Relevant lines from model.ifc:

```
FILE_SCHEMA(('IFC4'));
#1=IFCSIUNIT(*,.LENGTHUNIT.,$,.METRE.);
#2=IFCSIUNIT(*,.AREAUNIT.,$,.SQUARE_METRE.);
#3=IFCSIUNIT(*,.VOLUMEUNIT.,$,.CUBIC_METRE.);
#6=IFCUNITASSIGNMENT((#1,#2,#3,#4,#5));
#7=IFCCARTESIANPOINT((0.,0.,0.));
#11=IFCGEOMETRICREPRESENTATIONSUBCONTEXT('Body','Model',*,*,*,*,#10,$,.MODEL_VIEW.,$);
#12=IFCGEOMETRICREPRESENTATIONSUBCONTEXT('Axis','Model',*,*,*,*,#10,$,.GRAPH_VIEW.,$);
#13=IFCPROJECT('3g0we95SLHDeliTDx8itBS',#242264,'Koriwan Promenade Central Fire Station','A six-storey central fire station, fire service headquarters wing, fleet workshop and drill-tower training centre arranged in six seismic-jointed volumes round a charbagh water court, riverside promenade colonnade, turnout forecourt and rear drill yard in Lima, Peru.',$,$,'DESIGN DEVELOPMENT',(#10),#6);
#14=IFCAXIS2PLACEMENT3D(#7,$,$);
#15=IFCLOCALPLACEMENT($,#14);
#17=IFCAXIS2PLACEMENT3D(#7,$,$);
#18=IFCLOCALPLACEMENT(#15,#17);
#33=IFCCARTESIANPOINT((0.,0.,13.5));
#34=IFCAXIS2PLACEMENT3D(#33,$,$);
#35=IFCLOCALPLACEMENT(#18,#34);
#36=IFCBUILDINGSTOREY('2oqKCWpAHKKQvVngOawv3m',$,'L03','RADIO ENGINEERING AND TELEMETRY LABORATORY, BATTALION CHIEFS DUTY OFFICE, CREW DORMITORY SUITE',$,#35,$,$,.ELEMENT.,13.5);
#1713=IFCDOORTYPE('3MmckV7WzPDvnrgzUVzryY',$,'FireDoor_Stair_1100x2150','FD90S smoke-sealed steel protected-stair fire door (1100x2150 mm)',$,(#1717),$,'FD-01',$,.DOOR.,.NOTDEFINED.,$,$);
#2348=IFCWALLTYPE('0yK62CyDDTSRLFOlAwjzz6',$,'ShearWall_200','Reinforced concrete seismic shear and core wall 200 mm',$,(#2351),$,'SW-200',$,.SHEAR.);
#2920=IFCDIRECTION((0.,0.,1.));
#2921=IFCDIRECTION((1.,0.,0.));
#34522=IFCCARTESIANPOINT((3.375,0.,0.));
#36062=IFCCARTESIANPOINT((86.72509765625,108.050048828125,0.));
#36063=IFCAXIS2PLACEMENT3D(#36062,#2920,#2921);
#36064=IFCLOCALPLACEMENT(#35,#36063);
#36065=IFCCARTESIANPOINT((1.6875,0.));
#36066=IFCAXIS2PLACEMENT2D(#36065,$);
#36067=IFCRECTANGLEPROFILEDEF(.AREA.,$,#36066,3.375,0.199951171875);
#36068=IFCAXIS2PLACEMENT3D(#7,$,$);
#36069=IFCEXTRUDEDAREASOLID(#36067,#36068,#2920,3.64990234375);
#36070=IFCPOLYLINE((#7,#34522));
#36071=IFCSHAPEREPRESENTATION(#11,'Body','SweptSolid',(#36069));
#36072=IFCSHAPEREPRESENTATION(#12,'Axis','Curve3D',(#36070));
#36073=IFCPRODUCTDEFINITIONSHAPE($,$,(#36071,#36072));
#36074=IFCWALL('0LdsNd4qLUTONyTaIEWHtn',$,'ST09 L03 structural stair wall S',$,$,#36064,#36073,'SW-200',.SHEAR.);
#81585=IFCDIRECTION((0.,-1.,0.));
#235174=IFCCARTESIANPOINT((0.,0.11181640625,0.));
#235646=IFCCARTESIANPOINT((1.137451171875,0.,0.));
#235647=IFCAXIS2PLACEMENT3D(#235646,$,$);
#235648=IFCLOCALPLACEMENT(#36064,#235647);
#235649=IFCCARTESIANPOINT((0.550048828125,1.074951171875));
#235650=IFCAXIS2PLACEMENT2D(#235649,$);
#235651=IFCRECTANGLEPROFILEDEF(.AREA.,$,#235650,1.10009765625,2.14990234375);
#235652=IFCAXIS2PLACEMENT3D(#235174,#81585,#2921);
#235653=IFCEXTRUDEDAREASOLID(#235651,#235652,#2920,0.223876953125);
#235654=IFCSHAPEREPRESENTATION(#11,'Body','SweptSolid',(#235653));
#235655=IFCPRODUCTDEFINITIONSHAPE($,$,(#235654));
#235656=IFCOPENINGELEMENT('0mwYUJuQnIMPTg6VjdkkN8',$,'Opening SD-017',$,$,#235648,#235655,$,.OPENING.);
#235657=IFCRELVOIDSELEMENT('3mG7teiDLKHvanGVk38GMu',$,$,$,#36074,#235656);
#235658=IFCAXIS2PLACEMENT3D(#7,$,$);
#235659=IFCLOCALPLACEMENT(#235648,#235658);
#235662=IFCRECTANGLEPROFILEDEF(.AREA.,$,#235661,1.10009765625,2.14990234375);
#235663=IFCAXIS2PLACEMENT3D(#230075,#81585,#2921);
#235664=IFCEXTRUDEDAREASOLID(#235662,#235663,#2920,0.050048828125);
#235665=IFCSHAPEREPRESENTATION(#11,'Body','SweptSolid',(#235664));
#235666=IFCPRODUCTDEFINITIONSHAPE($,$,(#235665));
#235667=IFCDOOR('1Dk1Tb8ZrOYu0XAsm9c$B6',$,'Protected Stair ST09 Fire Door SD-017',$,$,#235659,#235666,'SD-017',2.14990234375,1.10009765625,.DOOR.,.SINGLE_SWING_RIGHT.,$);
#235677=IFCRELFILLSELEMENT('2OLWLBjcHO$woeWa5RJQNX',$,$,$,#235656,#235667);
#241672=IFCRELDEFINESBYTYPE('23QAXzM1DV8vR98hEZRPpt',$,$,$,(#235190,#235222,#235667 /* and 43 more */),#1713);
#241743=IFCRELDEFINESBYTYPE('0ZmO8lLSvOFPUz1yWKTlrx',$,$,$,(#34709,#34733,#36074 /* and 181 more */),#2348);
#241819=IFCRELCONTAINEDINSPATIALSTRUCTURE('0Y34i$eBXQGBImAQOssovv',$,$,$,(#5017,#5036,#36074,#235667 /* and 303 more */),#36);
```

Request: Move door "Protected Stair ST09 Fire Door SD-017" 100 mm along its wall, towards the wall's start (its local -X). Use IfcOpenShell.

```python
import ifcopenshell
import ifcopenshell.api.geometry
import ifcopenshell.util.placement

model = ifcopenshell.open("model.ifc")

door = model.by_id(235667)
opening = door.FillsVoids[0].RelatingOpeningElement
wall = opening.VoidsElements[0].RelatingBuildingElement

wall_matrix = ifcopenshell.util.placement.get_local_placement(wall.ObjectPlacement)
shift = wall_matrix[:3, 0] * -0.1
before = ifcopenshell.util.placement.get_local_placement(door.ObjectPlacement)[:3, 3].copy()

# The door is placed relative to its opening, so it follows when the opening moves.
matrix = ifcopenshell.util.placement.get_local_placement(opening.ObjectPlacement)
matrix[:3, 3] += shift
ifcopenshell.api.geometry.edit_object_placement(
    model, product=opening, matrix=matrix, is_si=False, should_transform_children=True
)

after = ifcopenshell.util.placement.get_local_placement(door.ObjectPlacement)[:3, 3]
print("door moved by", (after - before).round(3) + 0.0)

model.write("model_updated.ifc")
```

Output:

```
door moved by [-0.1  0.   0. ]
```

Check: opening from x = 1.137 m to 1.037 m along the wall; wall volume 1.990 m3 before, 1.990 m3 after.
